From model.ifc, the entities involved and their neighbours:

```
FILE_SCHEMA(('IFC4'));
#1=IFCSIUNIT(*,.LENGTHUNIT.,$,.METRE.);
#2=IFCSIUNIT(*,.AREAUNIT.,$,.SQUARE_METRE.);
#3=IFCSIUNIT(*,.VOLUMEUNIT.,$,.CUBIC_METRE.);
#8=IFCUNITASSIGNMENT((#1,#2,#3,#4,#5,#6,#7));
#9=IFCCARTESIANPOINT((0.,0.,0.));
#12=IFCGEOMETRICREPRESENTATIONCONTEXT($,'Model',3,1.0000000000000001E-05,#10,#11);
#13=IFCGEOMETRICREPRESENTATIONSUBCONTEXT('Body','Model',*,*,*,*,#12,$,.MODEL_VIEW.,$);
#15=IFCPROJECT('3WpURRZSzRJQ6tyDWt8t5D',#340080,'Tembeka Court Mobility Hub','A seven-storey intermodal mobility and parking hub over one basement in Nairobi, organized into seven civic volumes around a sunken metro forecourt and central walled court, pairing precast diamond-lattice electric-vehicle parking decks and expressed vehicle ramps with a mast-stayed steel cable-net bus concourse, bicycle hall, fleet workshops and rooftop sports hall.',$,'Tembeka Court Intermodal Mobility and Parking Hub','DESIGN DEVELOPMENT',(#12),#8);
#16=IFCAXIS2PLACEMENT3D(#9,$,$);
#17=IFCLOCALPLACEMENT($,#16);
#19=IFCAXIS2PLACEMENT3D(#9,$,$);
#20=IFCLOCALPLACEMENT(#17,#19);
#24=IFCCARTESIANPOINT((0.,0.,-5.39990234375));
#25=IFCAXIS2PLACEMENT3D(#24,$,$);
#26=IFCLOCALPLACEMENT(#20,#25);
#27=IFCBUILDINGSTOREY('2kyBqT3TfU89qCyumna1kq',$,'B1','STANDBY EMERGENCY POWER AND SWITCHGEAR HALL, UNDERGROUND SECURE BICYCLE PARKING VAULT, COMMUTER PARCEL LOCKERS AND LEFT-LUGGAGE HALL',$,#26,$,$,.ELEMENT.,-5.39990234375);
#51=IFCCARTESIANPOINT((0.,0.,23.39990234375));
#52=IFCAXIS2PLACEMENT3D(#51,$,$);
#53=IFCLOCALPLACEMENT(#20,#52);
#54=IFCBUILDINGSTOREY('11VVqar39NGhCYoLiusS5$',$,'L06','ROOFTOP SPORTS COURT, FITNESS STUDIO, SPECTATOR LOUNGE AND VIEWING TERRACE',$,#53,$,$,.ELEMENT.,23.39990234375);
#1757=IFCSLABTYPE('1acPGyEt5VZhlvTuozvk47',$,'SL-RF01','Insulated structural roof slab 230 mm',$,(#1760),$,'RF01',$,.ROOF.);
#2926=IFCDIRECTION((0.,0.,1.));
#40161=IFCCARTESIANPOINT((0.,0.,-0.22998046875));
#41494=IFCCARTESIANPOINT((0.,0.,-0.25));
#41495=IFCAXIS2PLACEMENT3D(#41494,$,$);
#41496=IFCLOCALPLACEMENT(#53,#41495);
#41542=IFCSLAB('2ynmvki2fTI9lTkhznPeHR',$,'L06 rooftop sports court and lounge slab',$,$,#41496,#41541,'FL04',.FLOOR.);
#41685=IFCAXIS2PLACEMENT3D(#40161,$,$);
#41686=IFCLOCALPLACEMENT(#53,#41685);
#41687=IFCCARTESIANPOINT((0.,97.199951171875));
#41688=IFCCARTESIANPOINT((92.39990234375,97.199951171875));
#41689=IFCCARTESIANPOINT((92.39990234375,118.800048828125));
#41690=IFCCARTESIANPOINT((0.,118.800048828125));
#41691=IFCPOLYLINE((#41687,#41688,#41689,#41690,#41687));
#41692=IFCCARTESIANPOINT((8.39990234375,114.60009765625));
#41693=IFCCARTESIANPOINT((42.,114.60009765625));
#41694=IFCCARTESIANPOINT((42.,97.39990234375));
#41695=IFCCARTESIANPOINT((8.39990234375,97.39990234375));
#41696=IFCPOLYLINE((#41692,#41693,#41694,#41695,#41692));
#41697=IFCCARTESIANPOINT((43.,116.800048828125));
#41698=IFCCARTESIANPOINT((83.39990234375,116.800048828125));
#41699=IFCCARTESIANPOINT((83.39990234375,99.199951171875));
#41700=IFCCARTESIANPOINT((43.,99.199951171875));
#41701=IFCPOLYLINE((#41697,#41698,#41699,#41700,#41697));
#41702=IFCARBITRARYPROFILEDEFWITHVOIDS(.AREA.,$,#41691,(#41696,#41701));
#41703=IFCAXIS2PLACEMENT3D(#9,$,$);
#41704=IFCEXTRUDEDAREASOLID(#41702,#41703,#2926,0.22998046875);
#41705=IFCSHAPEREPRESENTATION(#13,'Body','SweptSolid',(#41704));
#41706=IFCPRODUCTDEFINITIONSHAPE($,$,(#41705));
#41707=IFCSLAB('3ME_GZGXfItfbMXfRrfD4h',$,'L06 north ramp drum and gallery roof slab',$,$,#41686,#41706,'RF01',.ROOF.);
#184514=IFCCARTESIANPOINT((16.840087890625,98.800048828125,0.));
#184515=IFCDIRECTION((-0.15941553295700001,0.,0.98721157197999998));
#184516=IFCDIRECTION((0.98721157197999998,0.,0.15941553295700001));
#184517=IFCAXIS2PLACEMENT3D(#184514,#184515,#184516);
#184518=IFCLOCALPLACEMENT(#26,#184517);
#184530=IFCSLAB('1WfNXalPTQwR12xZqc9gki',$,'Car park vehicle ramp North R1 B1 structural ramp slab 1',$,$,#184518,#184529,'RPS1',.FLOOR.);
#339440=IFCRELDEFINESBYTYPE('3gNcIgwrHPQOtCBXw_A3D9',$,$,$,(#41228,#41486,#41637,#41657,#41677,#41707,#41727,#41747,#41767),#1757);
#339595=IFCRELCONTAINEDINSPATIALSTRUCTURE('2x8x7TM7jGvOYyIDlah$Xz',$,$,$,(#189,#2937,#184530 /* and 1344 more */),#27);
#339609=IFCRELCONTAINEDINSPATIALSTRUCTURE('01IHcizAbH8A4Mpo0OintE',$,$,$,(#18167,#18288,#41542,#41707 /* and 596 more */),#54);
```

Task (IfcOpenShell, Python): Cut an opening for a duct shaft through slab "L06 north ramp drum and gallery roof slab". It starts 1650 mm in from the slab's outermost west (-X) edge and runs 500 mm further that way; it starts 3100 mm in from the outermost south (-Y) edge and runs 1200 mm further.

```python
import numpy as np
import ifcopenshell
import ifcopenshell.api.feature
import ifcopenshell.api.geometry
import ifcopenshell.api.root
import ifcopenshell.geom
import ifcopenshell.util.placement
import ifcopenshell.util.representation
import ifcopenshell.util.shape
import ifcopenshell.util.unit

model = ifcopenshell.open("model.ifc")
unit_scale = ifcopenshell.util.unit.calculate_unit_scale(model)
settings = ifcopenshell.geom.settings()


def volume(element):
    """Net volume in cubic metres, openings subtracted."""
    shape = ifcopenshell.geom.create_shape(settings, element)
    return ifcopenshell.util.shape.get_volume(shape.geometry)


slab = model.by_guid("3ME_GZGXfItfbMXfRrfD4h")
before = volume(slab)

# Extent in the slab's own axes, in metres. The edges named are its -X and -Y sides.
slab_shape = ifcopenshell.geom.create_shape(settings, slab)
vertices = ifcopenshell.util.shape.get_vertices(slab_shape.geometry)
x_min, y_min, bottom = vertices.min(axis=0)
top = vertices[:, 2].max()

opening = ifcopenshell.api.root.create_entity(model, ifc_class="IfcOpeningElement", name="Duct shaft opening", predefined_type="OPENING")
context = ifcopenshell.util.representation.get_context(model, "Model", "Body", "MODEL_VIEW")
width, depth = 0.5, 1.2
outline = [(0.0, 0.0), (width, 0.0), (width, depth), (0.0, depth), (0.0, 0.0)]
# Overshoot both faces by 50 mm so the cut is clean.
shape = ifcopenshell.api.geometry.add_slab_representation(
    model, context=context, depth=top - bottom + 0.1, polyline=outline
)
ifcopenshell.api.geometry.assign_representation(model, product=opening, representation=shape)

matrix = ifcopenshell.util.placement.get_local_placement(slab.ObjectPlacement)
matrix[:, 3] = matrix @ np.append(np.array([x_min + 1.65, y_min + 3.1, bottom - 0.05]) / unit_scale, 1.0)
ifcopenshell.api.geometry.edit_object_placement(model, product=opening, matrix=matrix, is_si=False)
ifcopenshell.api.feature.add_feature(model, feature=opening, element=slab)

after = volume(slab)

print(f"slab volume {before:.3f} -> {after:.3f} m3")

model.write("model_updated.ifc")
```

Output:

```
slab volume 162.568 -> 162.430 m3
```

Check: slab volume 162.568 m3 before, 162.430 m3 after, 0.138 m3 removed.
